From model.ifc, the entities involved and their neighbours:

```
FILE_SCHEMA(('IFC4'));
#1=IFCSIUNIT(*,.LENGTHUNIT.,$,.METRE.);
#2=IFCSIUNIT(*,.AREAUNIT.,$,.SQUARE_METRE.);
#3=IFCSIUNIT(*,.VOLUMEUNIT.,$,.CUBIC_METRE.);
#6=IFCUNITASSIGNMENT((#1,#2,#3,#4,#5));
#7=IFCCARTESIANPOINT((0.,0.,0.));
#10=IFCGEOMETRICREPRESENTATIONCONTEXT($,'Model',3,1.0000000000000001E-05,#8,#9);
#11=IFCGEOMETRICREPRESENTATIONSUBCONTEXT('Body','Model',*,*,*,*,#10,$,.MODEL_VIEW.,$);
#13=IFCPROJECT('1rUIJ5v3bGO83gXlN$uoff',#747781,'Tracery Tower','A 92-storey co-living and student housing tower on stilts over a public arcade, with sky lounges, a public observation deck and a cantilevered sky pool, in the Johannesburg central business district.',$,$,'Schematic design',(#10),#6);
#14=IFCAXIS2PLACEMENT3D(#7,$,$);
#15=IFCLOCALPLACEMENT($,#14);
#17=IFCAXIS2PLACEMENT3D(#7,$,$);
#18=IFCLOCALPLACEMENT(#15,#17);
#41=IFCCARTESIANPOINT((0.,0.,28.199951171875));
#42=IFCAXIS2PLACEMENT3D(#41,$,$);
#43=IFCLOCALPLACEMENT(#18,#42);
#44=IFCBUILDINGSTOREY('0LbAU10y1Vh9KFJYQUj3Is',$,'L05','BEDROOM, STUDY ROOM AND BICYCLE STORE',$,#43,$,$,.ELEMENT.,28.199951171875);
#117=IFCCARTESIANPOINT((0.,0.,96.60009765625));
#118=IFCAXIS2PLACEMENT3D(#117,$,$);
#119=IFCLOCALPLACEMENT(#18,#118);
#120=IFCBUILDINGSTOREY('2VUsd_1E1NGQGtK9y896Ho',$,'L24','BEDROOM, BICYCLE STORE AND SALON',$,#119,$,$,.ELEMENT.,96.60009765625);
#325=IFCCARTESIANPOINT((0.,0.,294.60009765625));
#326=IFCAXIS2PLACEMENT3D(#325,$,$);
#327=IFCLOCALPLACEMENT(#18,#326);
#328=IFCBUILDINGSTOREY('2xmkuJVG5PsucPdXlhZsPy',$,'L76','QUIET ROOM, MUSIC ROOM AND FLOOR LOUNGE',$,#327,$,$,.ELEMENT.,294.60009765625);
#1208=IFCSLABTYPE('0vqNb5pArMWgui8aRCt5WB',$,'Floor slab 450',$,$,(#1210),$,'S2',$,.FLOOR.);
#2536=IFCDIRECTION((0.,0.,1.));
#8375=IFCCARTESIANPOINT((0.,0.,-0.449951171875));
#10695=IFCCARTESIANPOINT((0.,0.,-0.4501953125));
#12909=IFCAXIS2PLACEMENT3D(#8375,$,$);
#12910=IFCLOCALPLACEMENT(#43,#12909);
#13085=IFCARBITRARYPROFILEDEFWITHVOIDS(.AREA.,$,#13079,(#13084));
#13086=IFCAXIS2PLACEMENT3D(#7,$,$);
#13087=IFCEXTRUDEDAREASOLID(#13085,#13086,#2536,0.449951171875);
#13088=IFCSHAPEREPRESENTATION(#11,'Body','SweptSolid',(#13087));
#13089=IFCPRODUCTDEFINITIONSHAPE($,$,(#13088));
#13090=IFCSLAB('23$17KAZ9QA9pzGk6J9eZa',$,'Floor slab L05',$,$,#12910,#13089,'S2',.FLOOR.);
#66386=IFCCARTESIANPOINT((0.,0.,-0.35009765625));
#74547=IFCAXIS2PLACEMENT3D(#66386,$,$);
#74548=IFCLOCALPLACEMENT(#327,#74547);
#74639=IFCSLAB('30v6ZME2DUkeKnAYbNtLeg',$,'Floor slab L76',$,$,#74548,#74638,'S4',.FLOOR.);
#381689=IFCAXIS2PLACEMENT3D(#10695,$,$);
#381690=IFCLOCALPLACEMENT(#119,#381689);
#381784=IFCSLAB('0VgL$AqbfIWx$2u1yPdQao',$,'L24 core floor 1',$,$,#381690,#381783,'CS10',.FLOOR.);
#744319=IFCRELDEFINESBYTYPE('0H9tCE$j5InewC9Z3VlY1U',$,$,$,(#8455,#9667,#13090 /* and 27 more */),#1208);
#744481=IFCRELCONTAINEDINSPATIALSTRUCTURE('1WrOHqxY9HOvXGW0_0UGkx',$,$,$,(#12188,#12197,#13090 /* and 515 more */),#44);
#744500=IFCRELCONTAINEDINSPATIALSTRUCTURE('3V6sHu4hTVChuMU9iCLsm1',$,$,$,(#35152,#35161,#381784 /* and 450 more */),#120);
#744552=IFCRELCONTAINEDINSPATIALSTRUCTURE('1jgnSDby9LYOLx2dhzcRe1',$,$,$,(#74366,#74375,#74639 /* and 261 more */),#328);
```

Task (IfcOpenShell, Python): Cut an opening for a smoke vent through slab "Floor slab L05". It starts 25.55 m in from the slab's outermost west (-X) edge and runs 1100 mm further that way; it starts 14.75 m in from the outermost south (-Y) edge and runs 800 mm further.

```python
import numpy as np
import ifcopenshell
import ifcopenshell.api.feature
import ifcopenshell.api.geometry
import ifcopenshell.api.root
import ifcopenshell.geom
import ifcopenshell.util.placement
import ifcopenshell.util.representation
import ifcopenshell.util.shape
import ifcopenshell.util.unit

model = ifcopenshell.open("model.ifc")
unit_scale = ifcopenshell.util.unit.calculate_unit_scale(model)
settings = ifcopenshell.geom.settings()


def volume(element):
    """Net volume in cubic metres, openings subtracted."""
    shape = ifcopenshell.geom.create_shape(settings, element)
    return ifcopenshell.util.shape.get_volume(shape.geometry)


slab = model.by_guid("23$17KAZ9QA9pzGk6J9eZa")
before = volume(slab)

# Extent in the slab's own axes, in metres. The edges named are its -X and -Y sides.
slab_shape = ifcopenshell.geom.create_shape(settings, slab)
vertices = ifcopenshell.util.shape.get_vertices(slab_shape.geometry)
x_min, y_min, bottom = vertices.min(axis=0)
top = vertices[:, 2].max()

opening = ifcopenshell.api.root.create_entity(model, ifc_class="IfcOpeningElement", name="Smoke vent opening", predefined_type="OPENING")
context = ifcopenshell.util.representation.get_context(model, "Model", "Body", "MODEL_VIEW")
width, depth = 1.1, 0.8
outline = [(0.0, 0.0), (width, 0.0), (width, depth), (0.0, depth), (0.0, 0.0)]
# Overshoot both faces by 50 mm so the cut is clean.
shape = ifcopenshell.api.geometry.add_slab_representation(
    model, context=context, depth=top - bottom + 0.1, polyline=outline
)
ifcopenshell.api.geometry.assign_representation(model, product=opening, representation=shape)

matrix = ifcopenshell.util.placement.get_local_placement(slab.ObjectPlacement)
matrix[:, 3] = matrix @ np.append(np.array([x_min + 25.55, y_min + 14.75, bottom - 0.05]) / unit_scale, 1.0)
ifcopenshell.api.geometry.edit_object_placement(model, product=opening, matrix=matrix, is_si=False)
ifcopenshell.api.feature.add_feature(model, feature=opening, element=slab)

after = volume(slab)

print(f"slab volume {before:.3f} -> {after:.3f} m3")

model.write("model_updated.ifc")
```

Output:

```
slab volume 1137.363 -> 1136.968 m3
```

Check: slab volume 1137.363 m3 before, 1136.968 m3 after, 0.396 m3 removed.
